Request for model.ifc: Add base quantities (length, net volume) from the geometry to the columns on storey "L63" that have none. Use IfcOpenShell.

First a look at what the model holds.

```python
import ifcopenshell
import ifcopenshell.util.element
import ifcopenshell.util.unit

model = ifcopenshell.open("model.ifc")
print(model.schema)
for unit_type in ("LENGTHUNIT", "AREAUNIT", "VOLUMEUNIT"):
    print(unit_type, ifcopenshell.util.unit.calculate_unit_scale(model, unit_type))
storey = next(s for s in model.by_type("IfcBuildingStorey") if s.Name == "L63")
columns = [e for e in ifcopenshell.util.element.get_decomposition(storey) if e.is_a("IfcColumn")]
for e in sorted(columns, key=lambda e: e.id()):
    print(e.id(), e.is_a(), e.Name, list(ifcopenshell.util.element.get_psets(e, qtos_only=True)), sep=" | ")
```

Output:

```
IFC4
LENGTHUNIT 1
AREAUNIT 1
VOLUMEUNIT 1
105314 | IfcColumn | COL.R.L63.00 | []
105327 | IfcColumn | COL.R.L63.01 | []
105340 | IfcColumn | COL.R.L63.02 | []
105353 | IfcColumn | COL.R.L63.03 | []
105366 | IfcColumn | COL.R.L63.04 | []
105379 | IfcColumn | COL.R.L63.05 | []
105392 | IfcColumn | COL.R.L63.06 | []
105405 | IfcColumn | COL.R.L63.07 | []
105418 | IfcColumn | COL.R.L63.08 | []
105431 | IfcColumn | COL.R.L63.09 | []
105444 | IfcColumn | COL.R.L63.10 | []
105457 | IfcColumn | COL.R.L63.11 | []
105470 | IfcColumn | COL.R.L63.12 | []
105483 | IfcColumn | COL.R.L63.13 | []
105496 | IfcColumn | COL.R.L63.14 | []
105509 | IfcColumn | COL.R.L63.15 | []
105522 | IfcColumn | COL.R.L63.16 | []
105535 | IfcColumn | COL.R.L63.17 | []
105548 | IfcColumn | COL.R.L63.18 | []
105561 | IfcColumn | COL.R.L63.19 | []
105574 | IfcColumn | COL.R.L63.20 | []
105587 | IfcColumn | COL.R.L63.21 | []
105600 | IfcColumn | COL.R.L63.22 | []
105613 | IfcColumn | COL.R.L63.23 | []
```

```python
import ifcopenshell
import ifcopenshell.api.pset
import ifcopenshell.geom
import ifcopenshell.util.element
import ifcopenshell.util.shape
import ifcopenshell.util.unit

model = ifcopenshell.open("model.ifc")
unit_scale = ifcopenshell.util.unit.calculate_unit_scale(model)
volume_scale = ifcopenshell.util.unit.calculate_unit_scale(model, "VOLUMEUNIT")
settings = ifcopenshell.geom.settings()

storey = next(s for s in model.by_type("IfcBuildingStorey") if s.Name == "L63")
columns = [e for e in ifcopenshell.util.element.get_decomposition(storey) if e.is_a("IfcColumn")]

for e in sorted(columns, key=lambda e: e.id()):
    if ifcopenshell.util.element.get_psets(e, qtos_only=True, should_inherit=False):
        continue
    # Geometry comes back in metres, in the element's own axes.
    shape = ifcopenshell.geom.create_shape(settings, e)
    values = {
        "Length": ifcopenshell.util.shape.get_z(shape.geometry) / unit_scale,
        "NetVolume": ifcopenshell.util.shape.get_volume(shape.geometry) / volume_scale,
    }
    qto = ifcopenshell.api.pset.add_qto(model, product=e, name="Qto_ColumnBaseQuantities")
    ifcopenshell.api.pset.edit_qto(model, qto=qto, properties=values)
    print(e.id(), {k: round(v, 3) for k, v in values.items()})

model.write("model-out.ifc")
```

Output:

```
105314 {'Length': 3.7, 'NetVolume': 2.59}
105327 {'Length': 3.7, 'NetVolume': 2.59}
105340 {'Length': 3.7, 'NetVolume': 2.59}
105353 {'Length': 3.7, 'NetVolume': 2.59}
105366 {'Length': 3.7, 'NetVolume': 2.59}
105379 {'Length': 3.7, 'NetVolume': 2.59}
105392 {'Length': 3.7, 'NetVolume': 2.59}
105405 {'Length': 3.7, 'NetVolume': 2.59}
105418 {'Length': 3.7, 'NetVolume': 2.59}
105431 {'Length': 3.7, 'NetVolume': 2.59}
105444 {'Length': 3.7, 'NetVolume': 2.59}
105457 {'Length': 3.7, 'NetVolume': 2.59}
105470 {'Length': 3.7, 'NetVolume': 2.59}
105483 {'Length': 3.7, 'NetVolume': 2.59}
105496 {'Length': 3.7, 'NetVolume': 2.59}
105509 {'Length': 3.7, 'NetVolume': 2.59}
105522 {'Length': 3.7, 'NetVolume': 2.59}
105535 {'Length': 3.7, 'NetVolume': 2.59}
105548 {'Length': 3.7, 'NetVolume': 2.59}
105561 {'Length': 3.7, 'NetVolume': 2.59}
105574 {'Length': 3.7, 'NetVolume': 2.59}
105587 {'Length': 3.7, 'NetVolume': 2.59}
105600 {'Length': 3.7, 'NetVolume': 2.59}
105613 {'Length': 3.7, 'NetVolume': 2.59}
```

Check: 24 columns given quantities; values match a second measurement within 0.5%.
